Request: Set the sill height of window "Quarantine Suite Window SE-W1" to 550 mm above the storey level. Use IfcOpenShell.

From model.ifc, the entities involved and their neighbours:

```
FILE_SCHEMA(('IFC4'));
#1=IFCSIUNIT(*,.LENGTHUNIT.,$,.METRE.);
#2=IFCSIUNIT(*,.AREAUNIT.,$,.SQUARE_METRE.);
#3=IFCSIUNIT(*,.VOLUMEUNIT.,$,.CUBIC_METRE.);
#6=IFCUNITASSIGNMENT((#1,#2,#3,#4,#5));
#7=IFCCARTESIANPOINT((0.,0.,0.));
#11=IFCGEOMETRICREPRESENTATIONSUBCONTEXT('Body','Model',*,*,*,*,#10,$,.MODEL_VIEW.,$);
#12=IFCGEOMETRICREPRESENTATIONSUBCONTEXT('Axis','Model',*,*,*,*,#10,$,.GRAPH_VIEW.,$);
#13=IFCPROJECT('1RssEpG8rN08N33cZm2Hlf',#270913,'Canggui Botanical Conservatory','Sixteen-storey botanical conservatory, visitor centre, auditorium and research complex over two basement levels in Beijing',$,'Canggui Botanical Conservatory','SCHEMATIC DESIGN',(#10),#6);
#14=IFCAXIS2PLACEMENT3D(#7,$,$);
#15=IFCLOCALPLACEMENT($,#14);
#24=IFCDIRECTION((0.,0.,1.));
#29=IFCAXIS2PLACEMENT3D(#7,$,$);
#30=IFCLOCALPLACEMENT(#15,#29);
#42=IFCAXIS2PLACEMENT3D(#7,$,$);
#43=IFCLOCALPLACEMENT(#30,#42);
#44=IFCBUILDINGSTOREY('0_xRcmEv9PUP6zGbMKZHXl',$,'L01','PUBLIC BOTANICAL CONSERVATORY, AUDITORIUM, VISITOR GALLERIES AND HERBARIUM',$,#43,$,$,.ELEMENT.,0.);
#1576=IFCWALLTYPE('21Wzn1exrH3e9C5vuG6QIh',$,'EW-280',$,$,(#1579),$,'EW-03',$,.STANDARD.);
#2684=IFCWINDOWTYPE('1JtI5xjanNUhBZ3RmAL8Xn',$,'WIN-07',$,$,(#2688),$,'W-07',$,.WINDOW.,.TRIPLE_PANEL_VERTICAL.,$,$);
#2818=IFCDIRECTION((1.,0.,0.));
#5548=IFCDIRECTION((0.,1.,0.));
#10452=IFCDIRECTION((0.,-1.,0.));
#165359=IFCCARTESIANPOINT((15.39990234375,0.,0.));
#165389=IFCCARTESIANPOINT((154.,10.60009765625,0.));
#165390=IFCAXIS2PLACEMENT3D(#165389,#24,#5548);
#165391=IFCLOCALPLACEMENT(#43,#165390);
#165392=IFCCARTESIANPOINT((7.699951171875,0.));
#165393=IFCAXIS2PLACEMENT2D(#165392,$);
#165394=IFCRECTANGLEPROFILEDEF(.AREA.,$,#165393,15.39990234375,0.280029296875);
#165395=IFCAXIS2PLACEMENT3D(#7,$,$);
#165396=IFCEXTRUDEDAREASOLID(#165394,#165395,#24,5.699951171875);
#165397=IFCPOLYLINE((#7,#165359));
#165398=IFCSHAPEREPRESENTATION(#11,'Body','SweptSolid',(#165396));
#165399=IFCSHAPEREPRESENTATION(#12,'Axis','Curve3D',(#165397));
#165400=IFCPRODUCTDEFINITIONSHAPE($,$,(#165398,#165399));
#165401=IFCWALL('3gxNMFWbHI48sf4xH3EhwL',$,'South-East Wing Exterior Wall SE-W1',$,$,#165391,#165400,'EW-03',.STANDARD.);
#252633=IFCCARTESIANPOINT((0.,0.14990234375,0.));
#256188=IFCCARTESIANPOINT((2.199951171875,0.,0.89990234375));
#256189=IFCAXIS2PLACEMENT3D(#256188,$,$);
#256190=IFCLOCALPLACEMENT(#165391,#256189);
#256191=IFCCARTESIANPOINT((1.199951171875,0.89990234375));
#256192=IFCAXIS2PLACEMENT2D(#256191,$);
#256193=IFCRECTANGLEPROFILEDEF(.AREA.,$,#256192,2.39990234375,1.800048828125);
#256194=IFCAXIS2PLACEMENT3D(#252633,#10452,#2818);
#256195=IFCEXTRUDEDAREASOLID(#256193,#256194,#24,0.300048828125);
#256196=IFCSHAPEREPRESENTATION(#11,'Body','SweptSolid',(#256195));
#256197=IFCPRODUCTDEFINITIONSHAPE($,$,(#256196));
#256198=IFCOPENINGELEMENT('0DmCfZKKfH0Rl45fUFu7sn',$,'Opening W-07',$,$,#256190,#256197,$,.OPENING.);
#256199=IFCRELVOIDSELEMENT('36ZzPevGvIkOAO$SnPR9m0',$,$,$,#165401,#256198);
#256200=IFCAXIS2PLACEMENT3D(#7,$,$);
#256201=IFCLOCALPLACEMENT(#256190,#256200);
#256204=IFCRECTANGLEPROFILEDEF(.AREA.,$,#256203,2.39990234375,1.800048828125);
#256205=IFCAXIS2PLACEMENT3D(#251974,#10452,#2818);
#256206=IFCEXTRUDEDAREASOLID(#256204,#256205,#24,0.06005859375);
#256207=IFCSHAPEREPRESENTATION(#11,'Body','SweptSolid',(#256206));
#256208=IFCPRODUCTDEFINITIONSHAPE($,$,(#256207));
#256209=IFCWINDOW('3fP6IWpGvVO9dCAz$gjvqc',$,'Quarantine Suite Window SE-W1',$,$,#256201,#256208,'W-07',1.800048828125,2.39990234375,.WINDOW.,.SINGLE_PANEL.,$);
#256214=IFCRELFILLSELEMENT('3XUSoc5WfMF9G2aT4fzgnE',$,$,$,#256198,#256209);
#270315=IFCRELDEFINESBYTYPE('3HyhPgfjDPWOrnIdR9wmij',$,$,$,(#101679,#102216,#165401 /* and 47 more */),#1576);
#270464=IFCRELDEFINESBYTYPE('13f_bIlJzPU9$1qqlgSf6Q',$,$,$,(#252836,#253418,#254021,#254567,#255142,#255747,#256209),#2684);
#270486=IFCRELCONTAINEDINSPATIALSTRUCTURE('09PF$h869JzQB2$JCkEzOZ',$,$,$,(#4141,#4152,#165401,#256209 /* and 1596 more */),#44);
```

```python
import numpy as np
import ifcopenshell
import ifcopenshell.api.geometry
import ifcopenshell.geom
import ifcopenshell.util.element
import ifcopenshell.util.placement
import ifcopenshell.util.shape
import ifcopenshell.util.unit

model = ifcopenshell.open("model.ifc")
unit_scale = ifcopenshell.util.unit.calculate_unit_scale(model)

window = model.by_id(256209)
opening = window.FillsVoids[0].RelatingOpeningElement
storey = ifcopenshell.util.element.get_container(window, ifc_class="IfcBuildingStorey")
level = ifcopenshell.util.placement.get_local_placement(storey.ObjectPlacement)[2, 3]

# The opening's origin need not be at the sill, so measure its lowest point.
shape = ifcopenshell.geom.create_shape(ifcopenshell.geom.settings(), opening)
bottom = ifcopenshell.util.shape.get_shape_bottom_elevation(shape, shape.geometry) / unit_scale
dz = level + 0.55 / unit_scale - bottom

shift = np.array([0.0, 0.0, dz])
# The window is placed relative to its opening, so it follows when the opening moves.
matrix = ifcopenshell.util.placement.get_local_placement(opening.ObjectPlacement)
matrix[:3, 3] += shift
ifcopenshell.api.geometry.edit_object_placement(
    model, product=opening, matrix=matrix, is_si=False, should_transform_children=True
)

print(f"moved by {dz * unit_scale:+.3f} m")

model.write("model_edited.ifc")
```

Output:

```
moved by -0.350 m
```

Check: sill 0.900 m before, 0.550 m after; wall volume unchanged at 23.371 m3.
